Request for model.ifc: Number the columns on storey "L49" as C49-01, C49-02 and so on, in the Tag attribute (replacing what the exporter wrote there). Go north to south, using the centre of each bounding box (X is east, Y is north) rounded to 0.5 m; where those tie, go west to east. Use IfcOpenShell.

First a look at what the model holds.

```python
import ifcopenshell
import ifcopenshell.util.element
import ifcopenshell.util.placement

model = ifcopenshell.open("model.ifc")
print(model.schema)
storey = next(s for s in model.by_type("IfcBuildingStorey") if s.Name == "L49")
columns = [e for e in ifcopenshell.util.element.get_decomposition(storey) if e.is_a("IfcColumn")]
for e in sorted(columns, key=lambda e: e.id()):
    origin = ifcopenshell.util.placement.get_local_placement(e.ObjectPlacement)[:3, 3]
    print(e.id(), e.Tag, e.Name, origin.round(2) + 0.0, sep=" | ")
```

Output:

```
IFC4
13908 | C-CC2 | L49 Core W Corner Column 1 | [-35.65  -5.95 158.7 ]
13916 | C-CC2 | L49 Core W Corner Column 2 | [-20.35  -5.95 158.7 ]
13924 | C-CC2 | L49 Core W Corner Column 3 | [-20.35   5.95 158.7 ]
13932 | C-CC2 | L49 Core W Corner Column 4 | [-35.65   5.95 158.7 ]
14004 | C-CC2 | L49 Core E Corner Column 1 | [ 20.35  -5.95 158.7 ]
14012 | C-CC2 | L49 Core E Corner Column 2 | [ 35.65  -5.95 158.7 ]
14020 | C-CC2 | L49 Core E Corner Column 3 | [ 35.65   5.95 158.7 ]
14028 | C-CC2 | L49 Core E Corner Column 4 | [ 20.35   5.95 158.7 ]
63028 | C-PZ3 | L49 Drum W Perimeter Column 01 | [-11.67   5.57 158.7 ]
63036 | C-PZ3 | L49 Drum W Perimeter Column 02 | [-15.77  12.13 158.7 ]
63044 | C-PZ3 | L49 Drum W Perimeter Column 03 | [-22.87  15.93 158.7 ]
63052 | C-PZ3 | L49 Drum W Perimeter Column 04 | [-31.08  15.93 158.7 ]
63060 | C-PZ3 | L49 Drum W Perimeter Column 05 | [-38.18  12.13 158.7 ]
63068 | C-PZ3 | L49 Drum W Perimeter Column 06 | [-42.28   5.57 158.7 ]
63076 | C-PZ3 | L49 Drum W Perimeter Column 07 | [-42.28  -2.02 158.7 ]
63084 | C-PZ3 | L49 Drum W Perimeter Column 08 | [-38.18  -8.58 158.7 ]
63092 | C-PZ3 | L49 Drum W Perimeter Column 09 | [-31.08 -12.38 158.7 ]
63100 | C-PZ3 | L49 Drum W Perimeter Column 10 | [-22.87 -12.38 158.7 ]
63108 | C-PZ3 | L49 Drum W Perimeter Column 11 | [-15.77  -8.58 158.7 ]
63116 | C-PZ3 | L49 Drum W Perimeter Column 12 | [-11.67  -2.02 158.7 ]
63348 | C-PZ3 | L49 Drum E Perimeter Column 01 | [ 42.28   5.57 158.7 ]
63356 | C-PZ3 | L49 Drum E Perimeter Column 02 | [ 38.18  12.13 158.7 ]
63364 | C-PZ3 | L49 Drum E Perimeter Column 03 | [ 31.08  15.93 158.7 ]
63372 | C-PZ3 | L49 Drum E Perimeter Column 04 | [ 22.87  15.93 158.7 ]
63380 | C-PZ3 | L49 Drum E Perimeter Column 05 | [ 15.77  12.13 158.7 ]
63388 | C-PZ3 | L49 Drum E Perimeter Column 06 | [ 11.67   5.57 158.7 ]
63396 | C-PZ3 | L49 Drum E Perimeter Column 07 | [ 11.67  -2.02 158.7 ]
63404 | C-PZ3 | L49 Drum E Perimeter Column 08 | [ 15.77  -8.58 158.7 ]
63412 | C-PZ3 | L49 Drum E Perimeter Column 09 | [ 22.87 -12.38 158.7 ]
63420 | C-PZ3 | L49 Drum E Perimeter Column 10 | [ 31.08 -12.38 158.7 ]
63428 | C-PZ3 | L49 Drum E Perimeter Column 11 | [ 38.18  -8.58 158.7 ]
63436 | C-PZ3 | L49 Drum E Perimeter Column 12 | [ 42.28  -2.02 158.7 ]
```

```python
import ifcopenshell
import ifcopenshell.geom
import ifcopenshell.util.element
import ifcopenshell.util.shape

model = ifcopenshell.open("model.ifc")
settings = ifcopenshell.geom.settings()
settings.set("use-world-coords", True)


def centre(element):
    shape = ifcopenshell.geom.create_shape(settings, element)
    return ifcopenshell.util.shape.get_bbox_centroid(shape.geometry)


storey = next(s for s in model.by_type("IfcBuildingStorey") if s.Name == "L49")
columns = [e for e in ifcopenshell.util.element.get_decomposition(storey) if e.is_a("IfcColumn")]

# Insertion points can sit at a corner or the storey origin, so sort by the geometry (in metres).
centres = {e: centre(e) for e in columns}
columns.sort(key=lambda e: (-round(centres[e][1] / 0.5), centres[e][0]))

for i, e in enumerate(columns, start=1):
    number = f"C49-{i:02d}"
    e.Tag = number
    print(e.id(), number)

model.write("model_v2.ifc")
```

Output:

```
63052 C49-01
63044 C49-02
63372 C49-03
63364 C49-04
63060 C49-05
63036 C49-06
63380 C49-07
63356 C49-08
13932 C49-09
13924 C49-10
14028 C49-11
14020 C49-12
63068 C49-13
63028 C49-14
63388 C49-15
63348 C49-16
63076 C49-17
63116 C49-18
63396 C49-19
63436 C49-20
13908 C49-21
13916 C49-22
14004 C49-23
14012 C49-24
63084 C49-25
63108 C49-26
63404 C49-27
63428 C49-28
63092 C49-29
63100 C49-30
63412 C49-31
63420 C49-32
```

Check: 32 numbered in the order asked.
